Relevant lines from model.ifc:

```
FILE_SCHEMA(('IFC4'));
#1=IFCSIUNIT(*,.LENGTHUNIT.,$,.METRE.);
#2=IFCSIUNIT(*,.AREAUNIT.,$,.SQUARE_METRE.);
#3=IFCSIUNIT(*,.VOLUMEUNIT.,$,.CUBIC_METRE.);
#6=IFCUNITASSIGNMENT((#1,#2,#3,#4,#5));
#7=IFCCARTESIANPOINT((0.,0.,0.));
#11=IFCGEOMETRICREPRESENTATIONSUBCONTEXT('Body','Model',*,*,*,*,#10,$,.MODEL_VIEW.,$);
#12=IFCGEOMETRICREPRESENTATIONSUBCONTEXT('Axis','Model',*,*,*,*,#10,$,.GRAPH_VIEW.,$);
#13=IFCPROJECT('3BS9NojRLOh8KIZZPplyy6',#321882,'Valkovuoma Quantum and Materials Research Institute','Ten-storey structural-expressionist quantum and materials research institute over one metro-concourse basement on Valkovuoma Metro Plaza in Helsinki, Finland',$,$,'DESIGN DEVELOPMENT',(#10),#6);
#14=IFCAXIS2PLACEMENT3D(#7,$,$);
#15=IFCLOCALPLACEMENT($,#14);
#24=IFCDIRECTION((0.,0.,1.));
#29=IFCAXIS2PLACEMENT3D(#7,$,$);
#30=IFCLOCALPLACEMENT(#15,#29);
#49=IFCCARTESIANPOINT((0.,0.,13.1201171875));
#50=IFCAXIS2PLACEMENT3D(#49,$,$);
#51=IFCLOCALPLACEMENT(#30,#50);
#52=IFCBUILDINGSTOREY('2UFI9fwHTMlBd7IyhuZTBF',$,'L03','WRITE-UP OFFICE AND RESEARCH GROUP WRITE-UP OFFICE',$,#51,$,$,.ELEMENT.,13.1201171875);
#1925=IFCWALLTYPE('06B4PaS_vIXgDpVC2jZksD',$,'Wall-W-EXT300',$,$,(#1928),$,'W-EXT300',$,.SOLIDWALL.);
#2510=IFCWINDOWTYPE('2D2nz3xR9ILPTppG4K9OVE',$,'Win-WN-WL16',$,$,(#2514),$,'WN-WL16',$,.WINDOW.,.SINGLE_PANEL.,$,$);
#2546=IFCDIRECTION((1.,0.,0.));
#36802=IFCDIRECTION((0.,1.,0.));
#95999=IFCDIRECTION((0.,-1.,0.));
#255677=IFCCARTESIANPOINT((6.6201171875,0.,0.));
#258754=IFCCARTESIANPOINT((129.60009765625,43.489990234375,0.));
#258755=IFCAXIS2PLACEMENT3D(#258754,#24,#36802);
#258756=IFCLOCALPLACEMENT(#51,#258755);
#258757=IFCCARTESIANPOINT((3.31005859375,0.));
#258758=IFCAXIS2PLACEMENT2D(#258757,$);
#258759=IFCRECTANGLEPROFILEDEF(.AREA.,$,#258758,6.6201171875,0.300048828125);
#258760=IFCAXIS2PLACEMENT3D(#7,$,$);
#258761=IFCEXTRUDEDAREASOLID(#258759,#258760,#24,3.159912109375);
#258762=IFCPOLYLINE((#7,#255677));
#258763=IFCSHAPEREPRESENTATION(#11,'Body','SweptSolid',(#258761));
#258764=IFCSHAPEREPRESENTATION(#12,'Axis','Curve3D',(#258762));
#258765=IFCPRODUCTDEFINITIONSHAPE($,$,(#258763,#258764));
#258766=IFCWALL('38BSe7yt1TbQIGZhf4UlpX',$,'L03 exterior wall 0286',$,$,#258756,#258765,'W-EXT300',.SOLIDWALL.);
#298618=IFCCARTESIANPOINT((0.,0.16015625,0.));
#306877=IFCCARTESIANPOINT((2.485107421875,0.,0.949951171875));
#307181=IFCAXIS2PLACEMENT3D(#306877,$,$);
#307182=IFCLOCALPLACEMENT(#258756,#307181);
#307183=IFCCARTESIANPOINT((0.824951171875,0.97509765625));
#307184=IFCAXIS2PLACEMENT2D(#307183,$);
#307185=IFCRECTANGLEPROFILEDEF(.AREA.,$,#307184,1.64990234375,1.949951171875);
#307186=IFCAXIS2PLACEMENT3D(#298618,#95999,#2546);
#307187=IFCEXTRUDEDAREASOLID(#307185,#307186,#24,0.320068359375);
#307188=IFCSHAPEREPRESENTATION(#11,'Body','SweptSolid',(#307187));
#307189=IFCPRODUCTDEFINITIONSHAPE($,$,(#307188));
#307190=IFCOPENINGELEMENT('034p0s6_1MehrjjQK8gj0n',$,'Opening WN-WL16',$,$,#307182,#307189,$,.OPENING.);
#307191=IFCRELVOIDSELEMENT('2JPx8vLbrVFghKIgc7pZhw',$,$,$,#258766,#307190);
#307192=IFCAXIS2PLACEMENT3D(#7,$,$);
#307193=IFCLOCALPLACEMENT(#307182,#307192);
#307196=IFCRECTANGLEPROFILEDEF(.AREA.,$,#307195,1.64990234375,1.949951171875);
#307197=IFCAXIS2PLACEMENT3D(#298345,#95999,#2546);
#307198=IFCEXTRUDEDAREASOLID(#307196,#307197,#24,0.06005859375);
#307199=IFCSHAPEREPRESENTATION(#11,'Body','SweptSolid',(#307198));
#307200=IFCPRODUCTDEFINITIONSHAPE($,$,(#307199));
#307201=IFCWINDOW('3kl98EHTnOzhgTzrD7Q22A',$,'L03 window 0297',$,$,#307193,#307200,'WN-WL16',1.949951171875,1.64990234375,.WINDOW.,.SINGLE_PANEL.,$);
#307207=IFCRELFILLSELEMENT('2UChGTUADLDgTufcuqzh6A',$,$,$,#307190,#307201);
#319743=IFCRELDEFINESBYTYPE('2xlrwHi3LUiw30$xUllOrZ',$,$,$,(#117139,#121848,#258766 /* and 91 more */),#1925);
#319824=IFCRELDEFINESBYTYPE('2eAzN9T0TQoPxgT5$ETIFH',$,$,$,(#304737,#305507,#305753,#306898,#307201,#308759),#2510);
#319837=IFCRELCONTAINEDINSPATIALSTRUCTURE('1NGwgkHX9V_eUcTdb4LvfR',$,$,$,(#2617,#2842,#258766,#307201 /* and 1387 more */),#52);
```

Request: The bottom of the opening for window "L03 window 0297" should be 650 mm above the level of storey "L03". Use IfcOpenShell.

```python
import numpy as np
import ifcopenshell
import ifcopenshell.api.geometry
import ifcopenshell.geom
import ifcopenshell.util.element
import ifcopenshell.util.placement
import ifcopenshell.util.shape
import ifcopenshell.util.unit

model = ifcopenshell.open("model.ifc")
unit_scale = ifcopenshell.util.unit.calculate_unit_scale(model)

window = model.by_guid("3kl98EHTnOzhgTzrD7Q22A")
opening = window.FillsVoids[0].RelatingOpeningElement
storey = ifcopenshell.util.element.get_container(window, ifc_class="IfcBuildingStorey")
level = ifcopenshell.util.placement.get_local_placement(storey.ObjectPlacement)[2, 3]

# The opening's origin need not be at the sill, so measure its lowest point.
shape = ifcopenshell.geom.create_shape(ifcopenshell.geom.settings(), opening)
bottom = ifcopenshell.util.shape.get_shape_bottom_elevation(shape, shape.geometry) / unit_scale
dz = level + 0.65 / unit_scale - bottom

shift = np.array([0.0, 0.0, dz])
# The window is placed relative to its opening, so it follows when the opening moves.
matrix = ifcopenshell.util.placement.get_local_placement(opening.ObjectPlacement)
matrix[:3, 3] += shift
ifcopenshell.api.geometry.edit_object_placement(
    model, product=opening, matrix=matrix, is_si=False, should_transform_children=True
)

print(f"moved by {dz * unit_scale:+.3f} m")

model.write("model_v2.ifc")
```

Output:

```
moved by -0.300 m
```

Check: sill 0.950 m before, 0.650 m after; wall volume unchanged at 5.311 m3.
